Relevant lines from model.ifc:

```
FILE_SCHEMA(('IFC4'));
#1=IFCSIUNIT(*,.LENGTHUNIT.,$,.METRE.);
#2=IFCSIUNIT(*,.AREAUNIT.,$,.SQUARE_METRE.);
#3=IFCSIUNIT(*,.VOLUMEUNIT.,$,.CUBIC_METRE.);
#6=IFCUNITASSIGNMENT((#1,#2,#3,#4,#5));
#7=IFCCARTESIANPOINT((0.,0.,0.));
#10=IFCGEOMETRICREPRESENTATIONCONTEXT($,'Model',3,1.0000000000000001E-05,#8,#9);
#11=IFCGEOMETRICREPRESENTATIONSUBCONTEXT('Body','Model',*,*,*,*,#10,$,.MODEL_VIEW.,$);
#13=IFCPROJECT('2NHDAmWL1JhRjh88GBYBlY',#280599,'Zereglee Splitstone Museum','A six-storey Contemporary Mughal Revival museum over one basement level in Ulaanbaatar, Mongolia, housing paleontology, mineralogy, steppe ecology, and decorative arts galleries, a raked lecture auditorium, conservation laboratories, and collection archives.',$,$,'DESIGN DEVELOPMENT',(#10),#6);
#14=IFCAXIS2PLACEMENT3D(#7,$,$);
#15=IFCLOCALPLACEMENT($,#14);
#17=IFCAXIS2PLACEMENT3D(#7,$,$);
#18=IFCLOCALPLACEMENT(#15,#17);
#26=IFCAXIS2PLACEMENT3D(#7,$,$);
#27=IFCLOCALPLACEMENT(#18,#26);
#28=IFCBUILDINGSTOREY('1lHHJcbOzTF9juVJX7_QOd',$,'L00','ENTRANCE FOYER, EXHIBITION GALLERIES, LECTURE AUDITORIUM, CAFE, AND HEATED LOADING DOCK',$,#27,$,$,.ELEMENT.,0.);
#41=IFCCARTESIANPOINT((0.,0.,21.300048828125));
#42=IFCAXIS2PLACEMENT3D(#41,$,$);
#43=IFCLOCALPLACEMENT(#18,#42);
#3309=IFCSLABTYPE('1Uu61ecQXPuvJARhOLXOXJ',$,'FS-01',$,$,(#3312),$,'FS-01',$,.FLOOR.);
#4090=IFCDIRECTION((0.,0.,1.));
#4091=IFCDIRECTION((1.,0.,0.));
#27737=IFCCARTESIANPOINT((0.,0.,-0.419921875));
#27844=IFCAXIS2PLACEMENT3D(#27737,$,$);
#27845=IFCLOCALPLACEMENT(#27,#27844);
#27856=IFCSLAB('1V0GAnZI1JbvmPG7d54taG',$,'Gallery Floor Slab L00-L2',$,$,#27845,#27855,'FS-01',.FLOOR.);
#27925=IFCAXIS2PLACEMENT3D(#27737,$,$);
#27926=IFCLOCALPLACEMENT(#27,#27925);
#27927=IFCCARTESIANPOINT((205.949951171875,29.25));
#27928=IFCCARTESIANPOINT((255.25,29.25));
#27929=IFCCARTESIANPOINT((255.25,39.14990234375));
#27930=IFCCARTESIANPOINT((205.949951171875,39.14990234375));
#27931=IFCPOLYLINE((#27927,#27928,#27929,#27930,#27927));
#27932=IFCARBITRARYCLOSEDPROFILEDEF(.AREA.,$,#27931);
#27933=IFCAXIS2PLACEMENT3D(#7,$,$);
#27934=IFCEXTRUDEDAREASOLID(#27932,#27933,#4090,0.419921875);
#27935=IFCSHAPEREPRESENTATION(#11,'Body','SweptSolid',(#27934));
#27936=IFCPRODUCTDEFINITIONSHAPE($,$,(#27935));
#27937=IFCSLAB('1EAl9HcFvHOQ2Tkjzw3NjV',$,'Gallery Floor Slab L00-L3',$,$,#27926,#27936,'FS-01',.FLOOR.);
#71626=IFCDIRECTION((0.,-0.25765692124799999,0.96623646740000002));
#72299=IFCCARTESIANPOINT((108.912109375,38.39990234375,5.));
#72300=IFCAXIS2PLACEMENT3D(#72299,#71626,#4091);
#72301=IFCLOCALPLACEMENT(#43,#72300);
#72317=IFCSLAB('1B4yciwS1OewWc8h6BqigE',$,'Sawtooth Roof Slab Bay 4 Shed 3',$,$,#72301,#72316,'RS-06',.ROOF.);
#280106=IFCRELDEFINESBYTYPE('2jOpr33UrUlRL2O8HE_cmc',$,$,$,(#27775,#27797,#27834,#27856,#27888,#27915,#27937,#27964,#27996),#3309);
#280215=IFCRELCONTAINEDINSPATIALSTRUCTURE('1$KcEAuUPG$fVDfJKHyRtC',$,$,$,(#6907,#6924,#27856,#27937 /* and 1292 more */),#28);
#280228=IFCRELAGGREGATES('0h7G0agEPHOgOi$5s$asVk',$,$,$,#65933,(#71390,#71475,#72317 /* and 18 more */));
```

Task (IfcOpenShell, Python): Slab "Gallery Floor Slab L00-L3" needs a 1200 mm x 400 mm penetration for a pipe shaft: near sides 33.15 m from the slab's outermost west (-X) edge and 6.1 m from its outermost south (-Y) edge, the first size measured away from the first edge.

```python
import numpy as np
import ifcopenshell
import ifcopenshell.api.feature
import ifcopenshell.api.geometry
import ifcopenshell.api.root
import ifcopenshell.geom
import ifcopenshell.util.placement
import ifcopenshell.util.representation
import ifcopenshell.util.shape
import ifcopenshell.util.unit

model = ifcopenshell.open("model.ifc")
unit_scale = ifcopenshell.util.unit.calculate_unit_scale(model)
settings = ifcopenshell.geom.settings()


def volume(element):
    """Net volume in cubic metres, openings subtracted."""
    shape = ifcopenshell.geom.create_shape(settings, element)
    return ifcopenshell.util.shape.get_volume(shape.geometry)


slab = model.by_id(27937)
before = volume(slab)

# Extent in the slab's own axes, in metres. The edges named are its -X and -Y sides.
slab_shape = ifcopenshell.geom.create_shape(settings, slab)
vertices = ifcopenshell.util.shape.get_vertices(slab_shape.geometry)
x_min, y_min, bottom = vertices.min(axis=0)
top = vertices[:, 2].max()

opening = ifcopenshell.api.root.create_entity(model, ifc_class="IfcOpeningElement", name="Pipe shaft opening", predefined_type="OPENING")
context = ifcopenshell.util.representation.get_context(model, "Model", "Body", "MODEL_VIEW")
width, depth = 1.2, 0.4
outline = [(0.0, 0.0), (width, 0.0), (width, depth), (0.0, depth), (0.0, 0.0)]
# Overshoot both faces by 50 mm so the cut is clean.
shape = ifcopenshell.api.geometry.add_slab_representation(
    model, context=context, depth=top - bottom + 0.1, polyline=outline
)
ifcopenshell.api.geometry.assign_representation(model, product=opening, representation=shape)

matrix = ifcopenshell.util.placement.get_local_placement(slab.ObjectPlacement)
matrix[:, 3] = matrix @ np.append(np.array([x_min + 33.15, y_min + 6.1, bottom - 0.05]) / unit_scale, 1.0)
ifcopenshell.api.geometry.edit_object_placement(model, product=opening, matrix=matrix, is_si=False)
ifcopenshell.api.feature.add_feature(model, feature=opening, element=slab)

after = volume(slab)

print(f"slab volume {before:.3f} -> {after:.3f} m3")

model.write("model-out.ifc")
```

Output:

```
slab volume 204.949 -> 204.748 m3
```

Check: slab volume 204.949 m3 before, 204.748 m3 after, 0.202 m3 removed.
